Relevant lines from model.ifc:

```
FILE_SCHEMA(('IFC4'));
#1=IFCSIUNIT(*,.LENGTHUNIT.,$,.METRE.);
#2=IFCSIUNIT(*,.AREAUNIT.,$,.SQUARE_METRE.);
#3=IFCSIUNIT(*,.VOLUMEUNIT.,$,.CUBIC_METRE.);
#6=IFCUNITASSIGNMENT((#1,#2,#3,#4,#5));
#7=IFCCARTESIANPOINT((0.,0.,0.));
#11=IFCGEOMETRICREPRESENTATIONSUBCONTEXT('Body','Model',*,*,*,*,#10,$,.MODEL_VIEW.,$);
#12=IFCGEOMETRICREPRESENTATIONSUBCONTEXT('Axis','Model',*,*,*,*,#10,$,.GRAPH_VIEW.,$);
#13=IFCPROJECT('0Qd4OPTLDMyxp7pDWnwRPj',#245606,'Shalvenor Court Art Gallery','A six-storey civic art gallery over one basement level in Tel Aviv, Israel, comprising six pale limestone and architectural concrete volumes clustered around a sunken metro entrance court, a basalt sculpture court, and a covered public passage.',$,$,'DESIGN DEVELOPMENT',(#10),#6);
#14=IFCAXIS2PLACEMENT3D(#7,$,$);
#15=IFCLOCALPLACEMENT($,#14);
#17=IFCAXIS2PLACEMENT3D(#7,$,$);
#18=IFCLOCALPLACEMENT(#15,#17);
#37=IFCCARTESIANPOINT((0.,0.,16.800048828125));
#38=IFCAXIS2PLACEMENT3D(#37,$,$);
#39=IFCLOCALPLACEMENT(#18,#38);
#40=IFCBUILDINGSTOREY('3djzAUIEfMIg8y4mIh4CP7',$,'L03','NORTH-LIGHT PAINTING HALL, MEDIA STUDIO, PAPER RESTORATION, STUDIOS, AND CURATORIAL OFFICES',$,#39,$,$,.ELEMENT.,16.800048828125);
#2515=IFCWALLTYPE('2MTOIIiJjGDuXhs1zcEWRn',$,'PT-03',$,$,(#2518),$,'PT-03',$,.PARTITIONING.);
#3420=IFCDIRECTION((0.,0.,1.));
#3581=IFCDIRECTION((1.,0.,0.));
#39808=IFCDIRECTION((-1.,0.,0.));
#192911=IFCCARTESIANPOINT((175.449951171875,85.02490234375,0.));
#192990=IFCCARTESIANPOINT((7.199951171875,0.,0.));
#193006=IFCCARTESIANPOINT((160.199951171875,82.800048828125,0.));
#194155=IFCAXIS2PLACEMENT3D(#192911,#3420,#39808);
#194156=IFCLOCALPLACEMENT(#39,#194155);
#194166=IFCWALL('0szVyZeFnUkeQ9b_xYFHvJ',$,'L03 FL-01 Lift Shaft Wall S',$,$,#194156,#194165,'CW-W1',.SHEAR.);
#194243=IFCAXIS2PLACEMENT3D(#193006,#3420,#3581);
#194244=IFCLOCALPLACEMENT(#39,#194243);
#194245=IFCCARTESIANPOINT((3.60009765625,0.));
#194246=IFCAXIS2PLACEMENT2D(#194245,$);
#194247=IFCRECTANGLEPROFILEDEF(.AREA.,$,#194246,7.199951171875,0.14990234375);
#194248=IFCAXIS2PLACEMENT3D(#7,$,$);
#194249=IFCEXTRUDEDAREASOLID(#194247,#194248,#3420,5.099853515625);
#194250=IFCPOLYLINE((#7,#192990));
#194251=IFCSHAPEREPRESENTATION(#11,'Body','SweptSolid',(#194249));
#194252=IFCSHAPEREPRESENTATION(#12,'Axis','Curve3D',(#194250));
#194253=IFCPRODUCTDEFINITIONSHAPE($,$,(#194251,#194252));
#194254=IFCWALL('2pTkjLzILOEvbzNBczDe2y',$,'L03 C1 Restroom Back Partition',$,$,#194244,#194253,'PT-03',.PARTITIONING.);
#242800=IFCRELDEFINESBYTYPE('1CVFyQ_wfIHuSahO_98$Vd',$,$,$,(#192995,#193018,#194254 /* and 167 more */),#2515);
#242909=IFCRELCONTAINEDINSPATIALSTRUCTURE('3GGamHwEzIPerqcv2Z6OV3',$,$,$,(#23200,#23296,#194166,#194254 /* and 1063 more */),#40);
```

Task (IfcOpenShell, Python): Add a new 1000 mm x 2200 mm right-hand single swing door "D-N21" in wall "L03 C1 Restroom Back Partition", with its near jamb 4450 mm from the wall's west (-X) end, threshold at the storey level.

```python
import numpy as np
import ifcopenshell
import ifcopenshell.api.feature
import ifcopenshell.api.geometry
import ifcopenshell.api.root
import ifcopenshell.api.spatial
import ifcopenshell.geom
import ifcopenshell.util.element
import ifcopenshell.util.placement
import ifcopenshell.util.representation
import ifcopenshell.util.shape
import ifcopenshell.util.unit

model = ifcopenshell.open("model.ifc")
unit_scale = ifcopenshell.util.unit.calculate_unit_scale(model)
settings = ifcopenshell.geom.settings()


def volume(element):
    """Net volume in cubic metres, openings subtracted."""
    shape = ifcopenshell.geom.create_shape(settings, element)
    return ifcopenshell.util.shape.get_volume(shape.geometry)


wall = model.by_guid("2pTkjLzILOEvbzNBczDe2y")
storey = ifcopenshell.util.element.get_container(wall, ifc_class="IfcBuildingStorey")
context = ifcopenshell.util.representation.get_context(model, "Model", "Body", "MODEL_VIEW")
before = volume(wall)

width, height, from_end, sill = 1, 2.2, 4.45, 0.0  # metres

# The wall runs along its own X axis, and the end named is its -X end.
wall_shape = ifcopenshell.geom.create_shape(settings, wall)
x, y, z = ifcopenshell.util.shape.get_vertices(wall_shape.geometry).T
start = x.min() + from_end
face, thickness = float(y.min()), float(y.max() - y.min())
wall_matrix = ifcopenshell.util.placement.get_local_placement(wall.ObjectPlacement)
level = ifcopenshell.util.placement.get_local_placement(storey.ObjectPlacement)[2, 3]


def in_wall(x, y):
    """Placement at x, y metres in the wall's axes, at sill height."""
    matrix = wall_matrix.copy()
    matrix[:, 3] = wall_matrix @ np.array([x / unit_scale, y / unit_scale, 0.0, 1.0])
    matrix[2, 3] = level + sill / unit_scale
    return matrix


# Opening: a box that overshoots both wall faces by 50 mm.
opening = ifcopenshell.api.root.create_entity(model, ifc_class="IfcOpeningElement", predefined_type="OPENING")
box = ifcopenshell.api.geometry.add_wall_representation(
    model, context=context, length=width, height=height, thickness=thickness + 0.1
)
ifcopenshell.api.geometry.assign_representation(model, product=opening, representation=box)
ifcopenshell.api.geometry.edit_object_placement(model, product=opening, matrix=in_wall(start, face - 0.05), is_si=False)
ifcopenshell.api.feature.add_feature(model, feature=opening, element=wall)

door = ifcopenshell.api.root.create_entity(model, ifc_class="IfcDoor", name="D-N21", predefined_type="DOOR")
door.OverallWidth, door.OverallHeight = width / unit_scale, height / unit_scale
door.OperationType = "SINGLE_SWING_RIGHT"
body = ifcopenshell.api.geometry.add_door_representation(
    model,
    context=context,
    overall_width=door.OverallWidth,
    overall_height=door.OverallHeight,
    operation_type="SINGLE_SWING_RIGHT",
    lining_properties={"LiningDepth": thickness / unit_scale, "ThresholdDepth": thickness / unit_scale},
)
ifcopenshell.api.geometry.assign_representation(model, product=door, representation=body)
ifcopenshell.api.spatial.assign_container(model, products=[door], relating_structure=storey)
ifcopenshell.api.feature.add_filling(model, opening=opening, element=door)

# The lining spans the wall, so the door starts at the wall face.
ifcopenshell.api.geometry.edit_object_placement(model, product=door, matrix=in_wall(start, face), is_si=False)

after = volume(wall)

print(f"wall volume {before:.3f} -> {after:.3f} m3")

model.write("model_edited.ifc")
```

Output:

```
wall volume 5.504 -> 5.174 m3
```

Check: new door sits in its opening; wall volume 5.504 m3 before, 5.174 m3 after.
